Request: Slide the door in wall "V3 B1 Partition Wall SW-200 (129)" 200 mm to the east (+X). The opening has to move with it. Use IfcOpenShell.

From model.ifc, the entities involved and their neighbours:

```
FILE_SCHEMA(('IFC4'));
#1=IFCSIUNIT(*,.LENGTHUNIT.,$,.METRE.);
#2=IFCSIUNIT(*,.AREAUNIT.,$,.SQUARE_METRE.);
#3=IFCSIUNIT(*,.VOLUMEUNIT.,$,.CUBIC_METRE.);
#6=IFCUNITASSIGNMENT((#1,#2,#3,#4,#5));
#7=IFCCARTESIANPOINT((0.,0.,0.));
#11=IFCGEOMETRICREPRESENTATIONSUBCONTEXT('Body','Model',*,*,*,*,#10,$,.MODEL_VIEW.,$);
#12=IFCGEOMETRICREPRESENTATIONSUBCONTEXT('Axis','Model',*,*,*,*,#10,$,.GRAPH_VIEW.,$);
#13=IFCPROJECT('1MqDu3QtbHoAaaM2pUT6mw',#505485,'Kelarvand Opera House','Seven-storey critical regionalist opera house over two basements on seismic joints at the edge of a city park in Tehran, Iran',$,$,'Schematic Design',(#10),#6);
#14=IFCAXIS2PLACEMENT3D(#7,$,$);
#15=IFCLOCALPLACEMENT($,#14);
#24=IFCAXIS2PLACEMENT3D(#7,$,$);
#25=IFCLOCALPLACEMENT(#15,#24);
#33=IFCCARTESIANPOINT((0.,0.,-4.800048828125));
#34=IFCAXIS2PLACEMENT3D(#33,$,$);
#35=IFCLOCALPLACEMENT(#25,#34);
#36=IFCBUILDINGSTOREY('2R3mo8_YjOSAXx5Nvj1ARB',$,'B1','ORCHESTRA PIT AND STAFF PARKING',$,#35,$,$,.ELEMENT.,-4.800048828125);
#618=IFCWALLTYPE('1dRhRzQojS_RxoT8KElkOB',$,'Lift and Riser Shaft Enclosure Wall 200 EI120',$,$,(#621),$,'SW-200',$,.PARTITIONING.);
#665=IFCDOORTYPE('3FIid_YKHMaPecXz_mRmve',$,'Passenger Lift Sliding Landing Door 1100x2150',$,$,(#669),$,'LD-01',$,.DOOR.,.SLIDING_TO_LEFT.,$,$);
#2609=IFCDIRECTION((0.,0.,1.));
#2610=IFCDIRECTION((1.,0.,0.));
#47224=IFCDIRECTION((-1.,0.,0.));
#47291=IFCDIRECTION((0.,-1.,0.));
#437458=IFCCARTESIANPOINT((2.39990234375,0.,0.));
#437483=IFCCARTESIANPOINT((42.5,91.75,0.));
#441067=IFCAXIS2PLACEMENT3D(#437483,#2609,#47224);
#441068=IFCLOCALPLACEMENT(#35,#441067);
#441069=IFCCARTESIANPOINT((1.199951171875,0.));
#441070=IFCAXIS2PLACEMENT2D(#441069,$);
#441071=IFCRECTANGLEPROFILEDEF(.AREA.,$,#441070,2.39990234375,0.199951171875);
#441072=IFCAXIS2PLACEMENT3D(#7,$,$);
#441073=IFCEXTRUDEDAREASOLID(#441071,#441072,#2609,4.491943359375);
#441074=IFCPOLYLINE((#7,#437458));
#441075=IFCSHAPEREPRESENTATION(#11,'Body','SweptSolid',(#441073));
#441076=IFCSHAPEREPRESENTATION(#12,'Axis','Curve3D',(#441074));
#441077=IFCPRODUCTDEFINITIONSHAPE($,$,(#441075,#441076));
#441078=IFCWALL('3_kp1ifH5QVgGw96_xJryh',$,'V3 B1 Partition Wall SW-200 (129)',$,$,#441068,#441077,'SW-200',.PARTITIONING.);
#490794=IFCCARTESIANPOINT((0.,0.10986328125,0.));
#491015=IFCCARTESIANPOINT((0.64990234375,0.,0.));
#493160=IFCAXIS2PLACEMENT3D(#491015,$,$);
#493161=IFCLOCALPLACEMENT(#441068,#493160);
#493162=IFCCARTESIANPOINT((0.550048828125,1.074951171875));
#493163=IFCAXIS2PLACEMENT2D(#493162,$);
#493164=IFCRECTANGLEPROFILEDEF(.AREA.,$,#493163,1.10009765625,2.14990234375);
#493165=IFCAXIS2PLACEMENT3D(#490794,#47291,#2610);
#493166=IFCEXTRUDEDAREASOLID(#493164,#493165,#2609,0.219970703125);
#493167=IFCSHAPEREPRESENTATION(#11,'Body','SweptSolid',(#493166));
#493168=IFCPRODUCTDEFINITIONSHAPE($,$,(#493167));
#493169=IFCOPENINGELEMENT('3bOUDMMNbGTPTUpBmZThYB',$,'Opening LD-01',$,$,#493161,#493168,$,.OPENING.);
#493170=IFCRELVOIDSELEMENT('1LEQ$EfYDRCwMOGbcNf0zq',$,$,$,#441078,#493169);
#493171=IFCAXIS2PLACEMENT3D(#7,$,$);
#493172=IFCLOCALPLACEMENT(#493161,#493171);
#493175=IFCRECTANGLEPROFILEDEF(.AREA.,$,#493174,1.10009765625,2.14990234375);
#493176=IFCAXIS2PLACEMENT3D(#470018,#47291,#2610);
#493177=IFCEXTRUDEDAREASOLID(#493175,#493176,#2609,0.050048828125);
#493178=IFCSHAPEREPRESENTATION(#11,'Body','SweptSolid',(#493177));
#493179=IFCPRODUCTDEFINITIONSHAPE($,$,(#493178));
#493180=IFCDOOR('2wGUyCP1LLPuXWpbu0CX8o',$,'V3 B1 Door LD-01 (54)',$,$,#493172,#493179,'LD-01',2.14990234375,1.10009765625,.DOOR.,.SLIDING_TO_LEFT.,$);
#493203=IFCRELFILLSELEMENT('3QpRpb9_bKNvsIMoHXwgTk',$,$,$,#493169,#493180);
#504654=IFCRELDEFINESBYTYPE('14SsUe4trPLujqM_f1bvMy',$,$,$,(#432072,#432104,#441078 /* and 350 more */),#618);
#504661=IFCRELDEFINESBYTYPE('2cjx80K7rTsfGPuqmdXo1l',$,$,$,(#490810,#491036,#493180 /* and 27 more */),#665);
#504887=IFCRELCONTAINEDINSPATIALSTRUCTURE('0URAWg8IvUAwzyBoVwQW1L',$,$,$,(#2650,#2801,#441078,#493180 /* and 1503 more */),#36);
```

```python
import ifcopenshell
import ifcopenshell.api.geometry
import ifcopenshell.util.placement
import ifcopenshell.util.unit

model = ifcopenshell.open("model.ifc")
unit_scale = ifcopenshell.util.unit.calculate_unit_scale(model)

door = model.by_guid("2wGUyCP1LLPuXWpbu0CX8o")
opening = door.FillsVoids[0].RelatingOpeningElement
wall = opening.VoidsElements[0].RelatingBuildingElement

wall_matrix = ifcopenshell.util.placement.get_local_placement(wall.ObjectPlacement)
shift = wall_matrix[:3, 0] * -0.2 / unit_scale
before = ifcopenshell.util.placement.get_local_placement(door.ObjectPlacement)[:3, 3].copy()

# The door is placed relative to its opening, so it follows when the opening moves.
matrix = ifcopenshell.util.placement.get_local_placement(opening.ObjectPlacement)
matrix[:3, 3] += shift
ifcopenshell.api.geometry.edit_object_placement(
    model, product=opening, matrix=matrix, is_si=False, should_transform_children=True
)

after = ifcopenshell.util.placement.get_local_placement(door.ObjectPlacement)[:3, 3]
print("door moved by", (after - before).round(3) + 0.0)

model.write("model-out.ifc")
```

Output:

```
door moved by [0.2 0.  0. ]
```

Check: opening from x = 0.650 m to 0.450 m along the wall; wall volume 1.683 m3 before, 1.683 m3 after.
